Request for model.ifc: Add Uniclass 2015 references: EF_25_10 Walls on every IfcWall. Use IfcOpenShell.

First a look at what the model holds.

```python
import ifcopenshell

model = ifcopenshell.open("model.ifc")
print(model.schema)
print("classifications:", [c.Name for c in model.by_type("IfcClassification")])
for ifc_class in ("IfcDoor", "IfcRoof", "IfcStair", "IfcWall", "IfcWindow"):
    print(ifc_class, len(model.by_type(ifc_class)))
```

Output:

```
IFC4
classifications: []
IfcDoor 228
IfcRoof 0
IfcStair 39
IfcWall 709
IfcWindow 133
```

```python
import ifcopenshell
import ifcopenshell.api.classification

model = ifcopenshell.open("model.ifc")

system = ifcopenshell.api.classification.add_classification(model, classification="Uniclass 2015")

codes = {
    "IfcWall": ("EF_25_10", "Walls"),
}
for ifc_class, (code, name) in codes.items():
    products = model.by_type(ifc_class)
    ifcopenshell.api.classification.add_reference(
        model, products=products, classification=system, identification=code, name=name
    )
    print(code, len(products))

model.write("model_v2.ifc")
```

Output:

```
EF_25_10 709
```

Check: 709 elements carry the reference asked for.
